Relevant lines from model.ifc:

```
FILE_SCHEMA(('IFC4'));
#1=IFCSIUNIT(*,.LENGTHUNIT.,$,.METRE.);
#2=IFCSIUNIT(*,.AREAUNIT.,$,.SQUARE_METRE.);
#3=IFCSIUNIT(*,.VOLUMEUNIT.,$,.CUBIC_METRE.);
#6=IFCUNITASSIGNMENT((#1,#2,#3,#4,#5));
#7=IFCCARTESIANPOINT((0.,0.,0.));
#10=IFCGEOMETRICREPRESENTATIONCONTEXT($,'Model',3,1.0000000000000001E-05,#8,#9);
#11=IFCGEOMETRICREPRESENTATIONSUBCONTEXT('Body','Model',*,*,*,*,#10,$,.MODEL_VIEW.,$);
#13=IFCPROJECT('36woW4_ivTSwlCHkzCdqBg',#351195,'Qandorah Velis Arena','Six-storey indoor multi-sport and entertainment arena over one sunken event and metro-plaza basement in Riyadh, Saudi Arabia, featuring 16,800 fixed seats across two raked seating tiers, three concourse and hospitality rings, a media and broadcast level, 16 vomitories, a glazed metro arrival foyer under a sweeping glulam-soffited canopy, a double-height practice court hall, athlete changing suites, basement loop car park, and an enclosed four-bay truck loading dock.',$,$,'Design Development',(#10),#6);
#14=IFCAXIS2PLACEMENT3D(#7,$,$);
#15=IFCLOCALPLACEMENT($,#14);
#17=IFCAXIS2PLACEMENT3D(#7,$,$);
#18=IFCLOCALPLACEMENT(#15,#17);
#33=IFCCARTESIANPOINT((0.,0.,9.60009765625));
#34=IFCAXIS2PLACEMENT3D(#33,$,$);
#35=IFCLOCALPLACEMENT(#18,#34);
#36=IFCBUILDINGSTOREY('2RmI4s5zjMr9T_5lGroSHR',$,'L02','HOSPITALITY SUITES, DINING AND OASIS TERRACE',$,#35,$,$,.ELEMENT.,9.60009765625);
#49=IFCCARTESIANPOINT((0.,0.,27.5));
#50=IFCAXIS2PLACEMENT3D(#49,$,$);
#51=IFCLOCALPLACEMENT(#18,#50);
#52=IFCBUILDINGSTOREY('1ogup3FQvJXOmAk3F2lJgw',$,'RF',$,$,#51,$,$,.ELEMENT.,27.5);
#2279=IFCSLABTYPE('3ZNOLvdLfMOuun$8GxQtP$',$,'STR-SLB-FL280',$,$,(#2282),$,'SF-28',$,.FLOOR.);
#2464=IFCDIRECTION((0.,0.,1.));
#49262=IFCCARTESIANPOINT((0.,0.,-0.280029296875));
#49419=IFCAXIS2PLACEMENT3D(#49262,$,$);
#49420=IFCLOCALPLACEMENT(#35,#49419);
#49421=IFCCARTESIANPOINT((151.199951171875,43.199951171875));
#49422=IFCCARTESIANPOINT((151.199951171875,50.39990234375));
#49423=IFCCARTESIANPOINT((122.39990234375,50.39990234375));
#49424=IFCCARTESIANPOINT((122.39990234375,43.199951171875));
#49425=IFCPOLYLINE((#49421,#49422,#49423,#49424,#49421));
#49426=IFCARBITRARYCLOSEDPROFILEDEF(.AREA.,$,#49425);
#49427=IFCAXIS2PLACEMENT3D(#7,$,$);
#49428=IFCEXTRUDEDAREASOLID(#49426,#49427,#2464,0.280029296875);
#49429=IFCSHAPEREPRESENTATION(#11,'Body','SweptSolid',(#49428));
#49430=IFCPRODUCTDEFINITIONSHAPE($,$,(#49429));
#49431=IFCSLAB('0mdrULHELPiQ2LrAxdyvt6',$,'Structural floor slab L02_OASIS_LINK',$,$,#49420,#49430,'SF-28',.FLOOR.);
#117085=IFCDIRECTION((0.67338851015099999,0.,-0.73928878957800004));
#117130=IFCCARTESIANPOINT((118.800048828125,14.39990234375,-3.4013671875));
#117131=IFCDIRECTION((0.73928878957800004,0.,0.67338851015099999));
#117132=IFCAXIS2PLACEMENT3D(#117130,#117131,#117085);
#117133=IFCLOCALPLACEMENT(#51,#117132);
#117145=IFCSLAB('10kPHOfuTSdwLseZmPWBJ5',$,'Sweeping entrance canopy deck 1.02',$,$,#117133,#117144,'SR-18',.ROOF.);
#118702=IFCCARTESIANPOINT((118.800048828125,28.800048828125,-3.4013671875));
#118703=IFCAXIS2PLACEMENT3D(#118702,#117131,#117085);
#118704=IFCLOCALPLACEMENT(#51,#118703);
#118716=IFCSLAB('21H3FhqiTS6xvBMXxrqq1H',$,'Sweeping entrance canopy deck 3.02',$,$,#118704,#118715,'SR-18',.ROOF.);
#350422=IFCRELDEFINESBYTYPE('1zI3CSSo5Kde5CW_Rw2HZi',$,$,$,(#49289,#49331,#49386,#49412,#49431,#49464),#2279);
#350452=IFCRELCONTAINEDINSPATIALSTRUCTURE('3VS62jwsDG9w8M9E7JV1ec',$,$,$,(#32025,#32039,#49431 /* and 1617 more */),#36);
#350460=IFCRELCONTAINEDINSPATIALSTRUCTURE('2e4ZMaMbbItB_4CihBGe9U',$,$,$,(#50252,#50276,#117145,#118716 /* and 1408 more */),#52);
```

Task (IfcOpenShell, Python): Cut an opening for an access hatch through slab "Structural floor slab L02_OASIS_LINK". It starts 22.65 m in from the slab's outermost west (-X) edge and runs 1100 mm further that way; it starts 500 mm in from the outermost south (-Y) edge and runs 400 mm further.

```python
import numpy as np
import ifcopenshell
import ifcopenshell.api.feature
import ifcopenshell.api.geometry
import ifcopenshell.api.root
import ifcopenshell.geom
import ifcopenshell.util.placement
import ifcopenshell.util.representation
import ifcopenshell.util.shape
import ifcopenshell.util.unit

model = ifcopenshell.open("model.ifc")
unit_scale = ifcopenshell.util.unit.calculate_unit_scale(model)
settings = ifcopenshell.geom.settings()


def volume(element):
    """Net volume in cubic metres, openings subtracted."""
    shape = ifcopenshell.geom.create_shape(settings, element)
    return ifcopenshell.util.shape.get_volume(shape.geometry)


slab = model.by_guid("0mdrULHELPiQ2LrAxdyvt6")
before = volume(slab)

# Extent in the slab's own axes, in metres. The edges named are its -X and -Y sides.
slab_shape = ifcopenshell.geom.create_shape(settings, slab)
vertices = ifcopenshell.util.shape.get_vertices(slab_shape.geometry)
x_min, y_min, bottom = vertices.min(axis=0)
top = vertices[:, 2].max()

opening = ifcopenshell.api.root.create_entity(model, ifc_class="IfcOpeningElement", name="Access hatch opening", predefined_type="OPENING")
context = ifcopenshell.util.representation.get_context(model, "Model", "Body", "MODEL_VIEW")
width, depth = 1.1, 0.4
outline = [(0.0, 0.0), (width, 0.0), (width, depth), (0.0, depth), (0.0, 0.0)]
# Overshoot both faces by 50 mm so the cut is clean.
shape = ifcopenshell.api.geometry.add_slab_representation(
    model, context=context, depth=top - bottom + 0.1, polyline=outline
)
ifcopenshell.api.geometry.assign_representation(model, product=opening, representation=shape)

matrix = ifcopenshell.util.placement.get_local_placement(slab.ObjectPlacement)
matrix[:, 3] = matrix @ np.append(np.array([x_min + 22.65, y_min + 0.5, bottom - 0.05]) / unit_scale, 1.0)
ifcopenshell.api.geometry.edit_object_placement(model, product=opening, matrix=matrix, is_si=False)
ifcopenshell.api.feature.add_feature(model, feature=opening, element=slab)

after = volume(slab)

print(f"slab volume {before:.3f} -> {after:.3f} m3")

model.write("model_edited.ifc")
```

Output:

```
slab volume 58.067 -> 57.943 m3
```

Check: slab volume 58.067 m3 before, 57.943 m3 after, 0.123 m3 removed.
